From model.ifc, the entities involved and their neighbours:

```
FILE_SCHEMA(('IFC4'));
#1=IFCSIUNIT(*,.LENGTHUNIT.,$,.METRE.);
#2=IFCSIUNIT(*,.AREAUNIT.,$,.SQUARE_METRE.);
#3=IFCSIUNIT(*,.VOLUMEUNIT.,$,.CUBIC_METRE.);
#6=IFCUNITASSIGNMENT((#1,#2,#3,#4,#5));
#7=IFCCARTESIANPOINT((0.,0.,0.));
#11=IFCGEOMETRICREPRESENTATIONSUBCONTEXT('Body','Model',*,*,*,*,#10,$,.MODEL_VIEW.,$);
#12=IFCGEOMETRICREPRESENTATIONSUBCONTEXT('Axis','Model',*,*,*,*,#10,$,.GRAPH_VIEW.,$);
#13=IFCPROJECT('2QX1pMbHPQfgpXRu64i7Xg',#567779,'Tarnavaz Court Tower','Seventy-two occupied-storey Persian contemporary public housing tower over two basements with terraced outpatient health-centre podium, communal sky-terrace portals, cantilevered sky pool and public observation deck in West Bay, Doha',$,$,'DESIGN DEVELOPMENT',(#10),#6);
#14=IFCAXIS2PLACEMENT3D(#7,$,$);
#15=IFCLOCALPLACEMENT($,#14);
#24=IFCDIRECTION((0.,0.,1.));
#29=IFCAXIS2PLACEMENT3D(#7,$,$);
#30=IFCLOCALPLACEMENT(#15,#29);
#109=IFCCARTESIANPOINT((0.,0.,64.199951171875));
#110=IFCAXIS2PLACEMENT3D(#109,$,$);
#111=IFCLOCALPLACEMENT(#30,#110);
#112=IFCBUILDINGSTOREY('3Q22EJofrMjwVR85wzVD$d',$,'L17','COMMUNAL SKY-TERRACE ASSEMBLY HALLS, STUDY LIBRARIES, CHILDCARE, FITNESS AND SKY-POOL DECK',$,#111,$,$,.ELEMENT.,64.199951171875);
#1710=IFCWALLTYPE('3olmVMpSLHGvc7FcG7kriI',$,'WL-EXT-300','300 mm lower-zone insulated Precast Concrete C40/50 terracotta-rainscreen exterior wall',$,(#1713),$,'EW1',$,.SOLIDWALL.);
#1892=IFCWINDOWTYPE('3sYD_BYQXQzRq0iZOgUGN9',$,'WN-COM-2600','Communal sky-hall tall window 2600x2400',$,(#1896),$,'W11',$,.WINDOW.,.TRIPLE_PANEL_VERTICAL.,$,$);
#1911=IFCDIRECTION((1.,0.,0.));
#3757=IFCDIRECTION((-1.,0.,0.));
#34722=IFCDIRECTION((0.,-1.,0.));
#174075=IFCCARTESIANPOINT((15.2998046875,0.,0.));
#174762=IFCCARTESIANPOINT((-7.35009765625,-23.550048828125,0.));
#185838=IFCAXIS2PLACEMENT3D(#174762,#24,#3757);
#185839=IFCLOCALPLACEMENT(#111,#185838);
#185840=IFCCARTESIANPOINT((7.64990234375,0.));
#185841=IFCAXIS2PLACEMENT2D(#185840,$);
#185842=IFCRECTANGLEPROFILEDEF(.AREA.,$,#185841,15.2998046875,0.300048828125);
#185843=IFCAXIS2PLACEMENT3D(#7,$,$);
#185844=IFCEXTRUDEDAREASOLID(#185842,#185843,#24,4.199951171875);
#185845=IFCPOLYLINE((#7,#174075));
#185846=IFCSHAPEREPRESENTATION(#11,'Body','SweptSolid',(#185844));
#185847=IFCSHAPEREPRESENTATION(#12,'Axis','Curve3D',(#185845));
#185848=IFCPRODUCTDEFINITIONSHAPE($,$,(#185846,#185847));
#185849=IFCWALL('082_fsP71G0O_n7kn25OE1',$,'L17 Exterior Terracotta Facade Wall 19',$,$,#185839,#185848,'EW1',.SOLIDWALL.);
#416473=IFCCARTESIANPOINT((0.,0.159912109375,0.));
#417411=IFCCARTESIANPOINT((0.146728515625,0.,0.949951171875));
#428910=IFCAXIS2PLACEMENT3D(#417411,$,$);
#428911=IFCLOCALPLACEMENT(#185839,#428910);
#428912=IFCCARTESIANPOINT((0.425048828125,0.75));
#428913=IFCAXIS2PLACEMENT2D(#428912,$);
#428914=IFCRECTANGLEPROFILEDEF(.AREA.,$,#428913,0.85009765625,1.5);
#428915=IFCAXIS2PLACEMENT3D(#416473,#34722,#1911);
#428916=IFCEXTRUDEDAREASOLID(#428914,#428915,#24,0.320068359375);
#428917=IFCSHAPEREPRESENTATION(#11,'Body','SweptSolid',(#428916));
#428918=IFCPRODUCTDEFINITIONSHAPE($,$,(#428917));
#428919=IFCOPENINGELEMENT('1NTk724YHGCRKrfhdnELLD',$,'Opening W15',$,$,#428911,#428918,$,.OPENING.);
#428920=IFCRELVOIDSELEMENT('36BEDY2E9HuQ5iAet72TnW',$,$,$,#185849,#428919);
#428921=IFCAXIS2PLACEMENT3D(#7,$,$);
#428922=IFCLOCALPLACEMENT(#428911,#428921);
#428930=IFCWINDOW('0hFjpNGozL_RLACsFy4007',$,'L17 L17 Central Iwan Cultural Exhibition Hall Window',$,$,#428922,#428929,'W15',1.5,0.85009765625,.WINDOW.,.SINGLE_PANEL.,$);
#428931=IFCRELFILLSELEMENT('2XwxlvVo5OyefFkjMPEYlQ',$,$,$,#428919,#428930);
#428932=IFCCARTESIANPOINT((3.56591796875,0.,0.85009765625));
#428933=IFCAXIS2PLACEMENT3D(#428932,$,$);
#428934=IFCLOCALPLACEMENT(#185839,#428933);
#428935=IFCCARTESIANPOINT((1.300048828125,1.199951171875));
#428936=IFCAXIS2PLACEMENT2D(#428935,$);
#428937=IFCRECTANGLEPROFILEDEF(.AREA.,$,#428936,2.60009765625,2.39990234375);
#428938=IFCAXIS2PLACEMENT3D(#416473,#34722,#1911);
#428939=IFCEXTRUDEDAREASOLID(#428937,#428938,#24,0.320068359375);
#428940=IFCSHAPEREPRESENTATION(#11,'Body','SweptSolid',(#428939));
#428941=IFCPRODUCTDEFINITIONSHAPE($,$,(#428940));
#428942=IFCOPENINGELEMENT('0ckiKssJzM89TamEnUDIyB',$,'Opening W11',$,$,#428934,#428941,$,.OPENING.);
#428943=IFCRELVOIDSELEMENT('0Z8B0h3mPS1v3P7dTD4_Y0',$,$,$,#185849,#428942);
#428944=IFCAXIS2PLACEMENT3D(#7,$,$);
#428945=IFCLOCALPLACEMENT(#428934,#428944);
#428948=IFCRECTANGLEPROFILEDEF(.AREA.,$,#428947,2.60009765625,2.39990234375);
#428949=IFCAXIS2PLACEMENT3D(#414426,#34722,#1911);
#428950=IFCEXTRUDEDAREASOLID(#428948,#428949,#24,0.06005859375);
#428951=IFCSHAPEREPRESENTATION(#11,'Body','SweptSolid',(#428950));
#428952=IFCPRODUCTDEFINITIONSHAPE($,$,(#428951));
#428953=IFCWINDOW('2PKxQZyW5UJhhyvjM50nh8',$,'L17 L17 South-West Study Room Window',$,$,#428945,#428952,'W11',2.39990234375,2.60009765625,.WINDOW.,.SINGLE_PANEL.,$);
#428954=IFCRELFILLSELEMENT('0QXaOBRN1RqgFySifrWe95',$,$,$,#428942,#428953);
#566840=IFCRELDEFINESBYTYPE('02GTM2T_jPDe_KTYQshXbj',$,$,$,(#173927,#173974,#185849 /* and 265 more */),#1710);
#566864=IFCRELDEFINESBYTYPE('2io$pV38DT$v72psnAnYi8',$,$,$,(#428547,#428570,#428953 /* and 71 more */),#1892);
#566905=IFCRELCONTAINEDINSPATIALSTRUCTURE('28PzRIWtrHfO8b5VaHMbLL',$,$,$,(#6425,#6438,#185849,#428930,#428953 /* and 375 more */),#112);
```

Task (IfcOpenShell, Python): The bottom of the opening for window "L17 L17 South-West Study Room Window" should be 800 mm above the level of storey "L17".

```python
import numpy as np
import ifcopenshell
import ifcopenshell.api.geometry
import ifcopenshell.geom
import ifcopenshell.util.element
import ifcopenshell.util.placement
import ifcopenshell.util.shape
import ifcopenshell.util.unit

model = ifcopenshell.open("model.ifc")
unit_scale = ifcopenshell.util.unit.calculate_unit_scale(model)

window = model.by_guid("2PKxQZyW5UJhhyvjM50nh8")
opening = window.FillsVoids[0].RelatingOpeningElement
storey = ifcopenshell.util.element.get_container(window, ifc_class="IfcBuildingStorey")
level = ifcopenshell.util.placement.get_local_placement(storey.ObjectPlacement)[2, 3]

# The opening's origin need not be at the sill, so measure its lowest point.
shape = ifcopenshell.geom.create_shape(ifcopenshell.geom.settings(), opening)
bottom = ifcopenshell.util.shape.get_shape_bottom_elevation(shape, shape.geometry) / unit_scale
dz = level + 0.8 / unit_scale - bottom

shift = np.array([0.0, 0.0, dz])
# The window is placed relative to its opening, so it follows when the opening moves.
matrix = ifcopenshell.util.placement.get_local_placement(opening.ObjectPlacement)
matrix[:3, 3] += shift
ifcopenshell.api.geometry.edit_object_placement(
    model, product=opening, matrix=matrix, is_si=False, should_transform_children=True
)

print(f"moved by {dz * unit_scale:+.3f} m")

model.write("model_updated.ifc")
```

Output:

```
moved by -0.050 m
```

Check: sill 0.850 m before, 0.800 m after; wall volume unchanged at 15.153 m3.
